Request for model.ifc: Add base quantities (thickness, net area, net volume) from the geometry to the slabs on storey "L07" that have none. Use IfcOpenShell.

First a look at what the model holds.

```python
import ifcopenshell
import ifcopenshell.util.element
import ifcopenshell.util.unit

model = ifcopenshell.open("model.ifc")
print(model.schema)
for unit_type in ("LENGTHUNIT", "AREAUNIT", "VOLUMEUNIT"):
    print(unit_type, ifcopenshell.util.unit.calculate_unit_scale(model, unit_type))
storey = next(s for s in model.by_type("IfcBuildingStorey") if s.Name == "L07")
slabs = [e for e in ifcopenshell.util.element.get_decomposition(storey) if e.is_a("IfcSlab")]
for e in sorted(slabs, key=lambda e: e.id()):
    print(e.id(), e.is_a(), e.Name, list(ifcopenshell.util.element.get_psets(e, qtos_only=True)), sep=" | ")
```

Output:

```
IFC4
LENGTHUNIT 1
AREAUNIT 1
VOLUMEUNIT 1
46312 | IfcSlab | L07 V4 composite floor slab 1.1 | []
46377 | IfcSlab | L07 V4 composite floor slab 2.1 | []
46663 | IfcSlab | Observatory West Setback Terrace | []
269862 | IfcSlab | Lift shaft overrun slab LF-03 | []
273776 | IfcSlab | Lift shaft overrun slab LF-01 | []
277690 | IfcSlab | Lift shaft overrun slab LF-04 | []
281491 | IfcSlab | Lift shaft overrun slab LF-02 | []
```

```python
import ifcopenshell
import ifcopenshell.api.pset
import ifcopenshell.geom
import ifcopenshell.util.element
import ifcopenshell.util.shape
import ifcopenshell.util.unit

model = ifcopenshell.open("model.ifc")
unit_scale = ifcopenshell.util.unit.calculate_unit_scale(model)
area_scale = ifcopenshell.util.unit.calculate_unit_scale(model, "AREAUNIT")
volume_scale = ifcopenshell.util.unit.calculate_unit_scale(model, "VOLUMEUNIT")
settings = ifcopenshell.geom.settings()

storey = next(s for s in model.by_type("IfcBuildingStorey") if s.Name == "L07")
slabs = [e for e in ifcopenshell.util.element.get_decomposition(storey) if e.is_a("IfcSlab")]

for e in sorted(slabs, key=lambda e: e.id()):
    if ifcopenshell.util.element.get_psets(e, qtos_only=True, should_inherit=False):
        continue
    # Geometry comes back in metres, in the element's own axes.
    shape = ifcopenshell.geom.create_shape(settings, e)
    values = {
        "Width": ifcopenshell.util.shape.get_z(shape.geometry) / unit_scale,
        "NetArea": ifcopenshell.util.shape.get_footprint_area(shape.geometry) / area_scale,
        "NetVolume": ifcopenshell.util.shape.get_volume(shape.geometry) / volume_scale,
    }
    qto = ifcopenshell.api.pset.add_qto(model, product=e, name="Qto_SlabBaseQuantities")
    ifcopenshell.api.pset.edit_qto(model, qto=qto, properties=values)
    print(e.id(), {k: round(v, 3) for k, v in values.items()})

model.write("model-out.ifc")
```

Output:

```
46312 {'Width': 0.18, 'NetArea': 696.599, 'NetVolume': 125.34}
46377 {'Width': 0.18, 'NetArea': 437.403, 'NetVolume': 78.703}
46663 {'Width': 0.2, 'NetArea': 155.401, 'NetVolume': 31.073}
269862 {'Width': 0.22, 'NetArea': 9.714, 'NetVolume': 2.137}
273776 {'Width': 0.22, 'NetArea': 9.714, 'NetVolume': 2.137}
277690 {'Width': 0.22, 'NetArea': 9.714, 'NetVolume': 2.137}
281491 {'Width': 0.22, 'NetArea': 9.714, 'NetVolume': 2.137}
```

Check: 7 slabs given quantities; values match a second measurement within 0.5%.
